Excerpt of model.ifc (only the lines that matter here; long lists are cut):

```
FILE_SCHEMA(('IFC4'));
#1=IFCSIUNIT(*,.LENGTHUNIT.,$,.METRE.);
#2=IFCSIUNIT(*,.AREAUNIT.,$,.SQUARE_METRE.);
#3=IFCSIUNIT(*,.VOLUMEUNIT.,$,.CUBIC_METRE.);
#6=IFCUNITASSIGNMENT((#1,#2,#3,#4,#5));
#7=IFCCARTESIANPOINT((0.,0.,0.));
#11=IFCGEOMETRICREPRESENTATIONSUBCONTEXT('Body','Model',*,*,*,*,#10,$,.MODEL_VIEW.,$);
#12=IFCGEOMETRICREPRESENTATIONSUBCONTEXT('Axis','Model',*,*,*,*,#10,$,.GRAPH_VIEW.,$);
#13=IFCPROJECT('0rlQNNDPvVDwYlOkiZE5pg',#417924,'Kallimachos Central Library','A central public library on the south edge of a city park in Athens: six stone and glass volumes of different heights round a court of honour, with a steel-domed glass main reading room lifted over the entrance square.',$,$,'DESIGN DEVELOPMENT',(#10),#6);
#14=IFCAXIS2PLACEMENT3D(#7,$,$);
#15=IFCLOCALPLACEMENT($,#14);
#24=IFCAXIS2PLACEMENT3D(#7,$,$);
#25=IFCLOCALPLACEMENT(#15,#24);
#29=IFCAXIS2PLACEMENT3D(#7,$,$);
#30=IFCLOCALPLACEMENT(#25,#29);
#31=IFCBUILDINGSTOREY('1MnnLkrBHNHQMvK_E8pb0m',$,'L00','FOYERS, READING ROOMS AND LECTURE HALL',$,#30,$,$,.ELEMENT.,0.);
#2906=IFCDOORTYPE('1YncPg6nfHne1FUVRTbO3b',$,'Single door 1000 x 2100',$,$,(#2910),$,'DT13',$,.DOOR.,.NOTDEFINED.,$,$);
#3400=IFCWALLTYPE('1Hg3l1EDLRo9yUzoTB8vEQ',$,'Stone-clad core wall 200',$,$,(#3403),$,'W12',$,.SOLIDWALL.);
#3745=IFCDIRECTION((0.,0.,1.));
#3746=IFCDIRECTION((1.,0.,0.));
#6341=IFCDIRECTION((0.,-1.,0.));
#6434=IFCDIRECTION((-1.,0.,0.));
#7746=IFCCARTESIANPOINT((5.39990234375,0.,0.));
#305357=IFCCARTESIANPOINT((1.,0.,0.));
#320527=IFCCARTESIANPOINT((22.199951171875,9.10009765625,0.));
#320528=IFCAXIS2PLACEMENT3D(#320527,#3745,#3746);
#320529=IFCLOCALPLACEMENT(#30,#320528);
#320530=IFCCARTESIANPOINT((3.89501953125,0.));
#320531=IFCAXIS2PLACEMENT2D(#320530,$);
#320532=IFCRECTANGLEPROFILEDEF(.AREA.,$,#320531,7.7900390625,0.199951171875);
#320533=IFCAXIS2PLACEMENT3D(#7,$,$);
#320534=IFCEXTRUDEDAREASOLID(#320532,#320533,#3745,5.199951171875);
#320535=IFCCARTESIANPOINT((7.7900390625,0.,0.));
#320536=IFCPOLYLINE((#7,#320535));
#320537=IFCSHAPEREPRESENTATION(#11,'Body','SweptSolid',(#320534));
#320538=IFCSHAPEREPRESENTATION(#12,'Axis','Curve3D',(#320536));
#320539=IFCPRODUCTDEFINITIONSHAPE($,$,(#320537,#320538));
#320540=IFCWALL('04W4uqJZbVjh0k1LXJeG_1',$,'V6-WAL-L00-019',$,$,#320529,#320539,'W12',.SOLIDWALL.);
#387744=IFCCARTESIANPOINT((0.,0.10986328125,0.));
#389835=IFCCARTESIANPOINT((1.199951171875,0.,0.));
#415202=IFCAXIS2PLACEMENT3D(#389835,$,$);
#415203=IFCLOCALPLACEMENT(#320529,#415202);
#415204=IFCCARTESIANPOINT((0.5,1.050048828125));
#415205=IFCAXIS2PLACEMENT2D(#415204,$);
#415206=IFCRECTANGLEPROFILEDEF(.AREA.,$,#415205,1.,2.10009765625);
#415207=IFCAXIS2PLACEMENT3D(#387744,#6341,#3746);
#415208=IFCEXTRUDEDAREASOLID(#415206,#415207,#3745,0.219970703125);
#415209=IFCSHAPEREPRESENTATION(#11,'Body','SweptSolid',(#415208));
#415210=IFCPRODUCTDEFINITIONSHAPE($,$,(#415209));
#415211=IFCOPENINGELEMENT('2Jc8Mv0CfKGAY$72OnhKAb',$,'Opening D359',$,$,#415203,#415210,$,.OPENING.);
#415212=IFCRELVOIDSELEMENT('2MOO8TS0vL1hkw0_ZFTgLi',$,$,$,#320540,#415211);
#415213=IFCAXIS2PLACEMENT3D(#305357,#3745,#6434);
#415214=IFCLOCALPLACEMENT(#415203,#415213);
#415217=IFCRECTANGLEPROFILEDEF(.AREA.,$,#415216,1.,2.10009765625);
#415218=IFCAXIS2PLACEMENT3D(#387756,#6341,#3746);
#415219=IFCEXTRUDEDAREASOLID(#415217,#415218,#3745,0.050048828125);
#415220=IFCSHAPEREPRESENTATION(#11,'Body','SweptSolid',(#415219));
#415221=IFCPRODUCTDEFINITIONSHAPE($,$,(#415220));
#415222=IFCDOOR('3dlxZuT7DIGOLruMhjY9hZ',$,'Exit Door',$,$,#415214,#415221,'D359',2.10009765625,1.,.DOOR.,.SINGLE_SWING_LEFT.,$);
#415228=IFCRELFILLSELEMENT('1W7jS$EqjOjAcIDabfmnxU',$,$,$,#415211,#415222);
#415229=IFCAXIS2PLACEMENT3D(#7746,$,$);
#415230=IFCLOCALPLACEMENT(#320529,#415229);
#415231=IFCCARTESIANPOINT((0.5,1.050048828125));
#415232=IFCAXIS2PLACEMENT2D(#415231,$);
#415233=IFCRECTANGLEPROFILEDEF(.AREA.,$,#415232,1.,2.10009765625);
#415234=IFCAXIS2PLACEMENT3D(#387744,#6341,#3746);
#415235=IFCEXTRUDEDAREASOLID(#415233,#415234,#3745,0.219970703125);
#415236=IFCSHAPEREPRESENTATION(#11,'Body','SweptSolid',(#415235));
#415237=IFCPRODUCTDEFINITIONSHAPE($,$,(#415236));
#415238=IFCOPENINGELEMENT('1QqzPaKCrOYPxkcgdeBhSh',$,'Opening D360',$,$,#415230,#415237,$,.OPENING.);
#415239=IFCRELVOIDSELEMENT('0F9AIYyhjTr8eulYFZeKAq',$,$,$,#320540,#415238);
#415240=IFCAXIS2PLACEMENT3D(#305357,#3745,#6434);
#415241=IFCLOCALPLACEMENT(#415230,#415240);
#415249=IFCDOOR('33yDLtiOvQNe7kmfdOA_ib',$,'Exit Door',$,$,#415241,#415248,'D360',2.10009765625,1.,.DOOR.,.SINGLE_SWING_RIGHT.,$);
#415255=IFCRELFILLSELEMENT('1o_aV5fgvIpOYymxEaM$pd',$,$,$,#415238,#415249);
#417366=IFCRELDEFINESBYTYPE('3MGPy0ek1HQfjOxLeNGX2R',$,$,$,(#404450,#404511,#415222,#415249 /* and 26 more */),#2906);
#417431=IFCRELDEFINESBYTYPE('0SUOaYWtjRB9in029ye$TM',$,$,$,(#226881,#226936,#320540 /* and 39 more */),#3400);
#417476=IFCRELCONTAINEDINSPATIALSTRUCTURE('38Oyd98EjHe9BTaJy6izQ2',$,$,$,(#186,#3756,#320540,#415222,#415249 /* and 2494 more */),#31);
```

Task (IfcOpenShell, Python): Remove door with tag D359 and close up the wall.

```python
import ifcopenshell
import ifcopenshell.api.feature
import ifcopenshell.api.root
import ifcopenshell.geom
import ifcopenshell.util.shape

model = ifcopenshell.open("model.ifc")
settings = ifcopenshell.geom.settings()


def volume(element):
    """Net volume in cubic metres, openings subtracted."""
    shape = ifcopenshell.geom.create_shape(settings, element)
    return ifcopenshell.util.shape.get_volume(shape.geometry)


door = model.by_guid("3dlxZuT7DIGOLruMhjY9hZ")
opening = door.FillsVoids[0].RelatingOpeningElement
wall = opening.VoidsElements[0].RelatingBuildingElement
before = volume(wall)

ifcopenshell.api.root.remove_product(model, product=door)
ifcopenshell.api.feature.remove_feature(model, feature=opening)

after = volume(wall)

print(f"wall volume {before:.3f} -> {after:.3f} m3")

model.write("model-out.ifc")
```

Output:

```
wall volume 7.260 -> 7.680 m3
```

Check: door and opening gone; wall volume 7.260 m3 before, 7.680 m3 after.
